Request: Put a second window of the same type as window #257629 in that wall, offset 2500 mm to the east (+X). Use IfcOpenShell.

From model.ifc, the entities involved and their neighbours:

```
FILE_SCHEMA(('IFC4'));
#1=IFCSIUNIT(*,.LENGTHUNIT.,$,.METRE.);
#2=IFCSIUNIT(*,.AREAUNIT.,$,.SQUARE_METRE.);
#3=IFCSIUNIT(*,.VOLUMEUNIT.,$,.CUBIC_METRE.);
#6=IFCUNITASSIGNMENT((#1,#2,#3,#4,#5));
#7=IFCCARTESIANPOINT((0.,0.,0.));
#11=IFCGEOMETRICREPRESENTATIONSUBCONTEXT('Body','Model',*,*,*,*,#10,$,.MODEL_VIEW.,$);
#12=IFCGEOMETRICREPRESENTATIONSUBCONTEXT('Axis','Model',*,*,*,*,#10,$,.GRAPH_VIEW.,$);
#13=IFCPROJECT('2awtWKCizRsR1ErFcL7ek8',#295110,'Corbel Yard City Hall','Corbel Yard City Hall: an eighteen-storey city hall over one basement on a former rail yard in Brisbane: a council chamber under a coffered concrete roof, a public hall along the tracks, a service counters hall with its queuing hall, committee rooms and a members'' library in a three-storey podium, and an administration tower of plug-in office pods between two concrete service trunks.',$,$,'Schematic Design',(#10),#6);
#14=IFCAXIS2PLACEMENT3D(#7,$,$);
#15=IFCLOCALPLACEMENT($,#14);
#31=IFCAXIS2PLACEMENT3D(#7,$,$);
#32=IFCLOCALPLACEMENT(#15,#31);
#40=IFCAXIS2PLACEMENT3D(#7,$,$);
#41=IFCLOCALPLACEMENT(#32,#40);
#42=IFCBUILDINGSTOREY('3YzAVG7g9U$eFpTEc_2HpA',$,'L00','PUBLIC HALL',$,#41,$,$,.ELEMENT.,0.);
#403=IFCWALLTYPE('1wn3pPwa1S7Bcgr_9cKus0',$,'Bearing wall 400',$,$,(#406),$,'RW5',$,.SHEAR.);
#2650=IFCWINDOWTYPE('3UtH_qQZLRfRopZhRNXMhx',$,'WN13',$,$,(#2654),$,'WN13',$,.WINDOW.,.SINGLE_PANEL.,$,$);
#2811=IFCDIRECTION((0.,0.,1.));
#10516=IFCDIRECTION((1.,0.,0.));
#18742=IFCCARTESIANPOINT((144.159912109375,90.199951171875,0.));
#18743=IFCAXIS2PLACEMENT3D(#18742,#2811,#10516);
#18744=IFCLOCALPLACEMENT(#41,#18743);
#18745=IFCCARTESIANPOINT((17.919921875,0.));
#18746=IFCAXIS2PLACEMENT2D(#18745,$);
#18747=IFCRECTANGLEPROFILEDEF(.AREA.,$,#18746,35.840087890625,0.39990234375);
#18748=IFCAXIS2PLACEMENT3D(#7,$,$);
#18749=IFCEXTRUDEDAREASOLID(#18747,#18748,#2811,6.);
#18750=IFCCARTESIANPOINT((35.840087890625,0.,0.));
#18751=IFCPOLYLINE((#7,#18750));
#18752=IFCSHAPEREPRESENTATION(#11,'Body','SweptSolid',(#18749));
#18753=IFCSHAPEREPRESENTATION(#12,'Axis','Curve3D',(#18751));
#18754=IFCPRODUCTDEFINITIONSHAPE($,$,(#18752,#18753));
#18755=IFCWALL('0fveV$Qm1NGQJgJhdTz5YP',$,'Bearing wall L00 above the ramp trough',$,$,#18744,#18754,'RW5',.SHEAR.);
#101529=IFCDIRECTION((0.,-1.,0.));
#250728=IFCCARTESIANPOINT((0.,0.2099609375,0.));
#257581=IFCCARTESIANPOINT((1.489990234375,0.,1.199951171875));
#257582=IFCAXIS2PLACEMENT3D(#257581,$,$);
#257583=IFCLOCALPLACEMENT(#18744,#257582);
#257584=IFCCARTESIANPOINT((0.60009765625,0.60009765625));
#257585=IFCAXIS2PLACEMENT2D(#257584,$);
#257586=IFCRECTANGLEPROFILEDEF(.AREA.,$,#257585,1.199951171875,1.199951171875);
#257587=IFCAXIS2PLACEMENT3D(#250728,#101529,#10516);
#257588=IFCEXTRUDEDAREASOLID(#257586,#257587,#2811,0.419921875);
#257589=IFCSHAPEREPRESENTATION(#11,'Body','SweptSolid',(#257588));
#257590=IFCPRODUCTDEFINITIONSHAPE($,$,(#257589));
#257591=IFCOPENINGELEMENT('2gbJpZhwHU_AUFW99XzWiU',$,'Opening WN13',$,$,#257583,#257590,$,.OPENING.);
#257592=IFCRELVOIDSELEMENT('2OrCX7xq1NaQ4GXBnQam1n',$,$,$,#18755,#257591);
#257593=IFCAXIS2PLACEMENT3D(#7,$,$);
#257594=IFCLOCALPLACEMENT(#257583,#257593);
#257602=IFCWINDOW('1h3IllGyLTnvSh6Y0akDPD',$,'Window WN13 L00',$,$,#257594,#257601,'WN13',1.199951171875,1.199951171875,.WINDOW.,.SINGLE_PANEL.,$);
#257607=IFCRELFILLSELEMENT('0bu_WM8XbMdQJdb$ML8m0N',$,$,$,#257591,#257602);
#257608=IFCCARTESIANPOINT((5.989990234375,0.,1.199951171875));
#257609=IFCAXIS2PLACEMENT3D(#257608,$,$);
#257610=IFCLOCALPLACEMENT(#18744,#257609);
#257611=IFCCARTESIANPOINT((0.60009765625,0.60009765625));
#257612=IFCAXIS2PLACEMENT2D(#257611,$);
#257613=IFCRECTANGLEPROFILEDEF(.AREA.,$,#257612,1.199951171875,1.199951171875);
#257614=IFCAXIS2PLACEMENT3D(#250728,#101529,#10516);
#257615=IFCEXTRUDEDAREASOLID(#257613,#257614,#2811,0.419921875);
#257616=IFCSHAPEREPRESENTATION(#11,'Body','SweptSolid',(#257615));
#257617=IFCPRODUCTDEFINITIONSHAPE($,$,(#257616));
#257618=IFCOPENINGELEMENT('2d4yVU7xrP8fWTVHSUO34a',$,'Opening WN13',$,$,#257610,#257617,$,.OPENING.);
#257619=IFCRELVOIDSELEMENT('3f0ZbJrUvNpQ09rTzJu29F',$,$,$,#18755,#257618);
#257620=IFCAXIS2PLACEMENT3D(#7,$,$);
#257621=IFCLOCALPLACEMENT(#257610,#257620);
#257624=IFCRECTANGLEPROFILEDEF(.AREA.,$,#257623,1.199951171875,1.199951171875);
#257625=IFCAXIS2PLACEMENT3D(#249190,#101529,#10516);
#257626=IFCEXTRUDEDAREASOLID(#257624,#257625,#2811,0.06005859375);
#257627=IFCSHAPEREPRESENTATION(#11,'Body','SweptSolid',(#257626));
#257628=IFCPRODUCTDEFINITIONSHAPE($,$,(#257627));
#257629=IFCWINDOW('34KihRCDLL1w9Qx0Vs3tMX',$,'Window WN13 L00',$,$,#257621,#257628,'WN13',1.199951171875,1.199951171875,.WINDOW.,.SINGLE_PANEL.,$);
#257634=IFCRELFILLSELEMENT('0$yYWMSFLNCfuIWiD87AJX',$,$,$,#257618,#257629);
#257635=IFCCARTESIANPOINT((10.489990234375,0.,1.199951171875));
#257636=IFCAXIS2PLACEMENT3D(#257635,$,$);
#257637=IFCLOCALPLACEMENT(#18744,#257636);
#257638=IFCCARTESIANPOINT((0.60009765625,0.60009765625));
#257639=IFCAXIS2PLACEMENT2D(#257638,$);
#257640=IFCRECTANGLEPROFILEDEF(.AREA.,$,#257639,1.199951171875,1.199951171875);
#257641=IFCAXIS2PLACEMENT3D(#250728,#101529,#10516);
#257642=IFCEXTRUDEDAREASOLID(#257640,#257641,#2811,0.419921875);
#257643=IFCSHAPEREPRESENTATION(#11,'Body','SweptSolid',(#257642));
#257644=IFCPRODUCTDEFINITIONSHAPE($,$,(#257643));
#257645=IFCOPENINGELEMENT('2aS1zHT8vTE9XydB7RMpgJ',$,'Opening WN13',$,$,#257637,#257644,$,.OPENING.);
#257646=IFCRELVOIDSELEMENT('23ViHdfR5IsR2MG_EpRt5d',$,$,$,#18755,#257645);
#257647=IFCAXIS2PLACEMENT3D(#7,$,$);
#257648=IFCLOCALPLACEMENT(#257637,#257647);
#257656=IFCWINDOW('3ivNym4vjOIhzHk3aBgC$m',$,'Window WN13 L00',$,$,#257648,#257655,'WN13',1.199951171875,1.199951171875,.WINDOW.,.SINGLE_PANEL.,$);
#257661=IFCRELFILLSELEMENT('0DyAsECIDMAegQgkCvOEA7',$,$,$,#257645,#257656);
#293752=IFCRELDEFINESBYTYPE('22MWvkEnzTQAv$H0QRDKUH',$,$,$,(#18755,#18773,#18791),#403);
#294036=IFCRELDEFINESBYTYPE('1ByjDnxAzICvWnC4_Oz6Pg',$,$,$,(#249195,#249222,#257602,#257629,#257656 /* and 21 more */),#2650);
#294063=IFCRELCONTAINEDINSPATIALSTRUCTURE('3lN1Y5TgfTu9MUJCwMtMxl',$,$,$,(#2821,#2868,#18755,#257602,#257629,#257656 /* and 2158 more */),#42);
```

```python
import ifcopenshell
import ifcopenshell.api.feature
import ifcopenshell.api.geometry
import ifcopenshell.api.root
import ifcopenshell.geom
import ifcopenshell.util.element
import ifcopenshell.util.placement
import ifcopenshell.util.shape

model = ifcopenshell.open("model.ifc")
settings = ifcopenshell.geom.settings()


def volume(element):
    """Net volume in cubic metres, openings subtracted."""
    shape = ifcopenshell.geom.create_shape(settings, element)
    return ifcopenshell.util.shape.get_volume(shape.geometry)


window = model.by_guid("34KihRCDLL1w9Qx0Vs3tMX")
opening = window.FillsVoids[0].RelatingOpeningElement
wall = opening.VoidsElements[0].RelatingBuildingElement
before = volume(wall)
shift = ifcopenshell.util.placement.get_local_placement(wall.ObjectPlacement)[:3, 0] * 2.5

# copy_class copies the void relationship, type, container and properties, but no geometry.
new_opening = ifcopenshell.api.root.copy_class(model, product=opening)
new_opening.Representation = ifcopenshell.util.element.copy_deep(
    model, opening.Representation, exclude=["IfcGeometricRepresentationContext", "IfcRepresentationMap"]
)
new_window = ifcopenshell.api.root.copy_class(model, product=window)
new_window.Representation = ifcopenshell.util.element.copy_deep(
    model, window.Representation, exclude=["IfcGeometricRepresentationContext", "IfcRepresentationMap"]
)
new_window.Tag = None
ifcopenshell.api.feature.add_filling(model, opening=new_opening, element=new_window)

for old, new in ((opening, new_opening), (window, new_window)):
    matrix = ifcopenshell.util.placement.get_local_placement(old.ObjectPlacement)
    matrix[:3, 3] += shift
    ifcopenshell.api.geometry.edit_object_placement(model, product=new, matrix=matrix, is_si=False)

after = volume(wall)

print(f"wall volume {before:.3f} -> {after:.3f} m3")

model.write("model_edited.ifc")
```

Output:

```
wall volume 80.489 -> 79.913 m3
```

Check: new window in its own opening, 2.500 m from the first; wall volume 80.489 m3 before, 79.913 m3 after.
